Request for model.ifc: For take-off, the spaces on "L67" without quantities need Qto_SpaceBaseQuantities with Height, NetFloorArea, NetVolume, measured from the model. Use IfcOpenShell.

First a look at what the model holds.

```python
import ifcopenshell
import ifcopenshell.util.element
import ifcopenshell.util.unit

model = ifcopenshell.open("model.ifc")
print(model.schema)
for unit_type in ("LENGTHUNIT", "AREAUNIT", "VOLUMEUNIT"):
    print(unit_type, ifcopenshell.util.unit.calculate_unit_scale(model, unit_type))
storey = next(s for s in model.by_type("IfcBuildingStorey") if s.Name == "L67")
spaces = [e for e in ifcopenshell.util.element.get_decomposition(storey) if e.is_a("IfcSpace")]
for e in sorted(spaces, key=lambda e: e.id()):
    print(e.id(), e.is_a(), e.Name, list(ifcopenshell.util.element.get_psets(e, qtos_only=True)), sep=" | ")
```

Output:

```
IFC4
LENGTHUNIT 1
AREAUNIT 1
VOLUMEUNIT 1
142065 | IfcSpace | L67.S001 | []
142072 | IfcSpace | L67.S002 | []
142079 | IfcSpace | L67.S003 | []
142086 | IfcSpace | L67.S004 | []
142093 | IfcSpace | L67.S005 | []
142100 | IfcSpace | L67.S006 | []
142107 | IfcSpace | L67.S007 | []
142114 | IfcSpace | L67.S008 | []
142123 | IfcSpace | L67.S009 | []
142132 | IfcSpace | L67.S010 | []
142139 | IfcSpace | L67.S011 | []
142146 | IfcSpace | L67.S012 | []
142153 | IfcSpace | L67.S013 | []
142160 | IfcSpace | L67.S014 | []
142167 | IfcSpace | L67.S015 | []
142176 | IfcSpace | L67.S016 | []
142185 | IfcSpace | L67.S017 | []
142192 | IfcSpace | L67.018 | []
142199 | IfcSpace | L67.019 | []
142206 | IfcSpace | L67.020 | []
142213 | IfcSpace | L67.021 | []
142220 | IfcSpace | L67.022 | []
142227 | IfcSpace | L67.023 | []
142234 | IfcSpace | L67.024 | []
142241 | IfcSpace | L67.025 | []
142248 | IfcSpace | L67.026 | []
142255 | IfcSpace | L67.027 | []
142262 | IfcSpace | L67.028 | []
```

```python
import ifcopenshell
import ifcopenshell.api.pset
import ifcopenshell.geom
import ifcopenshell.util.element
import ifcopenshell.util.shape
import ifcopenshell.util.unit

model = ifcopenshell.open("model.ifc")
unit_scale = ifcopenshell.util.unit.calculate_unit_scale(model)
area_scale = ifcopenshell.util.unit.calculate_unit_scale(model, "AREAUNIT")
volume_scale = ifcopenshell.util.unit.calculate_unit_scale(model, "VOLUMEUNIT")
settings = ifcopenshell.geom.settings()

storey = next(s for s in model.by_type("IfcBuildingStorey") if s.Name == "L67")
spaces = [e for e in ifcopenshell.util.element.get_decomposition(storey) if e.is_a("IfcSpace")]

for e in sorted(spaces, key=lambda e: e.id()):
    if ifcopenshell.util.element.get_psets(e, qtos_only=True, should_inherit=False):
        continue
    # Geometry comes back in metres, in the element's own axes.
    shape = ifcopenshell.geom.create_shape(settings, e)
    values = {
        "Height": ifcopenshell.util.shape.get_z(shape.geometry) / unit_scale,
        "NetFloorArea": ifcopenshell.util.shape.get_footprint_area(shape.geometry) / area_scale,
        "NetVolume": ifcopenshell.util.shape.get_volume(shape.geometry) / volume_scale,
    }
    qto = ifcopenshell.api.pset.add_qto(model, product=e, name="Qto_SpaceBaseQuantities")
    ifcopenshell.api.pset.edit_qto(model, qto=qto, properties=values)
    print(e.id(), {k: round(v, 3) for k, v in values.items()})

model.write("model_v2.ifc")
```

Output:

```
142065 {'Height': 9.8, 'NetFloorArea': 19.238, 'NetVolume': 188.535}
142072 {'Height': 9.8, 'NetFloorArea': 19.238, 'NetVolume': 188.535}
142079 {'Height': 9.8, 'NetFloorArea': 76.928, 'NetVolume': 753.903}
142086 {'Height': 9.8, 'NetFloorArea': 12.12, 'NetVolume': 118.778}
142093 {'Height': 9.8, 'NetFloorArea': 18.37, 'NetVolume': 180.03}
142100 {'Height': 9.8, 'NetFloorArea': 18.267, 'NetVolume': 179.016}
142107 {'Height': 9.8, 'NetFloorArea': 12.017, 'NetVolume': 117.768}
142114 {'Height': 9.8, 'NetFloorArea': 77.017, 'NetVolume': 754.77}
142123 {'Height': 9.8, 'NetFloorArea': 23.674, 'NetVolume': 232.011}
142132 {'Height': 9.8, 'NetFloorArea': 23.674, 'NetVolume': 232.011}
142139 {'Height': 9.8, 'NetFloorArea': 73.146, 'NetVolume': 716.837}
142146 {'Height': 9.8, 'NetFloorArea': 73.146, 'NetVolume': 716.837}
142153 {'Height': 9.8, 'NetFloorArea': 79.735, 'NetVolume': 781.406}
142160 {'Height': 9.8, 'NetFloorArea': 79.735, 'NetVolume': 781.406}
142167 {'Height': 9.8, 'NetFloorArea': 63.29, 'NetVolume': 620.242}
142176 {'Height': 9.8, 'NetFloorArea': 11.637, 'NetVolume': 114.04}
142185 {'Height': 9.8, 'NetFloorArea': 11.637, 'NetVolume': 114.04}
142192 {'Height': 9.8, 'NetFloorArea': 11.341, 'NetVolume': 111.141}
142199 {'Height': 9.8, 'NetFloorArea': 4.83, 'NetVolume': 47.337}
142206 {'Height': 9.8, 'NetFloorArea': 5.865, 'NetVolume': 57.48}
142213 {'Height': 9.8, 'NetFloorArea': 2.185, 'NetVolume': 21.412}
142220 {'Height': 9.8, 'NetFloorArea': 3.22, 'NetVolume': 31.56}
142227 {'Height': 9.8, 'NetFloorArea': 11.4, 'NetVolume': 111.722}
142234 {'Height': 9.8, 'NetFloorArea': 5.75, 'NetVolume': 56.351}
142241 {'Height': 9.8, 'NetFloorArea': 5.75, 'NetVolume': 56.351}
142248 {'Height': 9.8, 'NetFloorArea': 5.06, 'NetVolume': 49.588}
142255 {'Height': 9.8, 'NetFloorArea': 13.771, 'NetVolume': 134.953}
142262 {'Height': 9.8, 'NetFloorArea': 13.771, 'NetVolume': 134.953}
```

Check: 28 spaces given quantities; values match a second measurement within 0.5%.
